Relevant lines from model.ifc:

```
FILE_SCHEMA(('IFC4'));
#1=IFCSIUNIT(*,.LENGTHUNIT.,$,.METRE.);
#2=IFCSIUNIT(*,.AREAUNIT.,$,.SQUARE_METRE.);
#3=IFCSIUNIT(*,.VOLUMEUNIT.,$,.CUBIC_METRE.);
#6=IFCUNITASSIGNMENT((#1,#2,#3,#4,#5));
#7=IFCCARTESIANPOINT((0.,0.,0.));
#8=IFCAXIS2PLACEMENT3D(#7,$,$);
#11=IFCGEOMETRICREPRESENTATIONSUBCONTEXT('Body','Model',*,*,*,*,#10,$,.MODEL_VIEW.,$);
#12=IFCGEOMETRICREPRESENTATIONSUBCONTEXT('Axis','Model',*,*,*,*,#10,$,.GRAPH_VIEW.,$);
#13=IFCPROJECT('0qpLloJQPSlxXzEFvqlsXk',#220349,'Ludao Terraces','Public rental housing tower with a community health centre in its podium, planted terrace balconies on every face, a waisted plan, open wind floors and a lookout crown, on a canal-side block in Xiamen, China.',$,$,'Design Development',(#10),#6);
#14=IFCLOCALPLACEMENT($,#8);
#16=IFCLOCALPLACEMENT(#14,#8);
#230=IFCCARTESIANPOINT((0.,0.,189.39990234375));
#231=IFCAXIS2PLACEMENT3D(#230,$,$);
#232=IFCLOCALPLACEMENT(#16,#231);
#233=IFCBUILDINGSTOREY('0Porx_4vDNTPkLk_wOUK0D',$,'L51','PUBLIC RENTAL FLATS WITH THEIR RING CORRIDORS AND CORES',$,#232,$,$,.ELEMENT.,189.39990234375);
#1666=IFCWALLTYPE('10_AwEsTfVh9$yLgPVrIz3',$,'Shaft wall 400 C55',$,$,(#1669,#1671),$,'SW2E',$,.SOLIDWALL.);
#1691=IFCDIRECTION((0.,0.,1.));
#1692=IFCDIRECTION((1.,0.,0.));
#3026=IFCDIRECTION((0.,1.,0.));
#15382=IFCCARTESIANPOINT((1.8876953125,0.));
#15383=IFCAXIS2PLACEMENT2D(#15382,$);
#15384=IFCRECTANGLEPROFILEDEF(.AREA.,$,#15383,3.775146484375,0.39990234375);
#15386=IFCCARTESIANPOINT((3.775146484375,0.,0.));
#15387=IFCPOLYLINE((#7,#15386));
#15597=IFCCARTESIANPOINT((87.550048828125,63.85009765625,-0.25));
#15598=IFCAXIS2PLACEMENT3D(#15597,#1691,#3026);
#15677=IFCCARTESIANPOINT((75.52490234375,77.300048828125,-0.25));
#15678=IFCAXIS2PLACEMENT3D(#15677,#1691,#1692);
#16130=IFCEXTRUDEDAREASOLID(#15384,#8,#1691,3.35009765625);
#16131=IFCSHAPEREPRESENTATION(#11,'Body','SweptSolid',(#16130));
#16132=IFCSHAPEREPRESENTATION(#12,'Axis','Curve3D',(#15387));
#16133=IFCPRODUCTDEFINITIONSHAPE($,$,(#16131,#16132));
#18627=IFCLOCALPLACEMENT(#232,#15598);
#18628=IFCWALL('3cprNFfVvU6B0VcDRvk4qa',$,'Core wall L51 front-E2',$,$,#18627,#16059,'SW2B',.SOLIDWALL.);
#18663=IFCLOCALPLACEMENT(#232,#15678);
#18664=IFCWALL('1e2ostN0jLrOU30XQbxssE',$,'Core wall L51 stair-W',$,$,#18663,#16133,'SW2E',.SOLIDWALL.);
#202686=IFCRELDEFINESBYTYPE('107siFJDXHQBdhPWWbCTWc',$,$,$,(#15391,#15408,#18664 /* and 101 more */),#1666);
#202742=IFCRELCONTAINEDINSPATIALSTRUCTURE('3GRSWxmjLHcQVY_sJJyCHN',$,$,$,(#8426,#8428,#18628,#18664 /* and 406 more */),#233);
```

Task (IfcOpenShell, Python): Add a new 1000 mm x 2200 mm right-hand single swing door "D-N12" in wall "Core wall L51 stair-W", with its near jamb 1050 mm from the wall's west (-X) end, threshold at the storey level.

```python
import numpy as np
import ifcopenshell
import ifcopenshell.api.feature
import ifcopenshell.api.geometry
import ifcopenshell.api.root
import ifcopenshell.api.spatial
import ifcopenshell.geom
import ifcopenshell.util.element
import ifcopenshell.util.placement
import ifcopenshell.util.representation
import ifcopenshell.util.shape
import ifcopenshell.util.unit

model = ifcopenshell.open("model.ifc")
unit_scale = ifcopenshell.util.unit.calculate_unit_scale(model)
settings = ifcopenshell.geom.settings()


def volume(element):
    """Net volume in cubic metres, openings subtracted."""
    shape = ifcopenshell.geom.create_shape(settings, element)
    return ifcopenshell.util.shape.get_volume(shape.geometry)


wall = model.by_id(18664)
storey = ifcopenshell.util.element.get_container(wall, ifc_class="IfcBuildingStorey")
context = ifcopenshell.util.representation.get_context(model, "Model", "Body", "MODEL_VIEW")
before = volume(wall)

width, height, from_end, sill = 1, 2.2, 1.05, 0.0  # metres

# The wall runs along its own X axis, and the end named is its -X end.
wall_shape = ifcopenshell.geom.create_shape(settings, wall)
x, y, z = ifcopenshell.util.shape.get_vertices(wall_shape.geometry).T
start = x.min() + from_end
face, thickness = float(y.min()), float(y.max() - y.min())
wall_matrix = ifcopenshell.util.placement.get_local_placement(wall.ObjectPlacement)
level = ifcopenshell.util.placement.get_local_placement(storey.ObjectPlacement)[2, 3]


def in_wall(x, y):
    """Placement at x, y metres in the wall's axes, at sill height."""
    matrix = wall_matrix.copy()
    matrix[:, 3] = wall_matrix @ np.array([x / unit_scale, y / unit_scale, 0.0, 1.0])
    matrix[2, 3] = level + sill / unit_scale
    return matrix


# Opening: a box that overshoots both wall faces by 50 mm.
opening = ifcopenshell.api.root.create_entity(model, ifc_class="IfcOpeningElement", predefined_type="OPENING")
box = ifcopenshell.api.geometry.add_wall_representation(
    model, context=context, length=width, height=height, thickness=thickness + 0.1
)
ifcopenshell.api.geometry.assign_representation(model, product=opening, representation=box)
ifcopenshell.api.geometry.edit_object_placement(model, product=opening, matrix=in_wall(start, face - 0.05), is_si=False)
ifcopenshell.api.feature.add_feature(model, feature=opening, element=wall)

door = ifcopenshell.api.root.create_entity(model, ifc_class="IfcDoor", name="D-N12", predefined_type="DOOR")
door.OverallWidth, door.OverallHeight = width / unit_scale, height / unit_scale
door.OperationType = "SINGLE_SWING_RIGHT"
body = ifcopenshell.api.geometry.add_door_representation(
    model,
    context=context,
    overall_width=door.OverallWidth,
    overall_height=door.OverallHeight,
    operation_type="SINGLE_SWING_RIGHT",
    lining_properties={"LiningDepth": thickness / unit_scale, "ThresholdDepth": thickness / unit_scale},
)
ifcopenshell.api.geometry.assign_representation(model, product=door, representation=body)
ifcopenshell.api.spatial.assign_container(model, products=[door], relating_structure=storey)
ifcopenshell.api.feature.add_filling(model, opening=opening, element=door)

# The lining spans the wall, so the door starts at the wall face.
ifcopenshell.api.geometry.edit_object_placement(model, product=door, matrix=in_wall(start, face), is_si=False)

after = volume(wall)

print(f"wall volume {before:.3f} -> {after:.3f} m3")

model.write("model_rev.ifc")
```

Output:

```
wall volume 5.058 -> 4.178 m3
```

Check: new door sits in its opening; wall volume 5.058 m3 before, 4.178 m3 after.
